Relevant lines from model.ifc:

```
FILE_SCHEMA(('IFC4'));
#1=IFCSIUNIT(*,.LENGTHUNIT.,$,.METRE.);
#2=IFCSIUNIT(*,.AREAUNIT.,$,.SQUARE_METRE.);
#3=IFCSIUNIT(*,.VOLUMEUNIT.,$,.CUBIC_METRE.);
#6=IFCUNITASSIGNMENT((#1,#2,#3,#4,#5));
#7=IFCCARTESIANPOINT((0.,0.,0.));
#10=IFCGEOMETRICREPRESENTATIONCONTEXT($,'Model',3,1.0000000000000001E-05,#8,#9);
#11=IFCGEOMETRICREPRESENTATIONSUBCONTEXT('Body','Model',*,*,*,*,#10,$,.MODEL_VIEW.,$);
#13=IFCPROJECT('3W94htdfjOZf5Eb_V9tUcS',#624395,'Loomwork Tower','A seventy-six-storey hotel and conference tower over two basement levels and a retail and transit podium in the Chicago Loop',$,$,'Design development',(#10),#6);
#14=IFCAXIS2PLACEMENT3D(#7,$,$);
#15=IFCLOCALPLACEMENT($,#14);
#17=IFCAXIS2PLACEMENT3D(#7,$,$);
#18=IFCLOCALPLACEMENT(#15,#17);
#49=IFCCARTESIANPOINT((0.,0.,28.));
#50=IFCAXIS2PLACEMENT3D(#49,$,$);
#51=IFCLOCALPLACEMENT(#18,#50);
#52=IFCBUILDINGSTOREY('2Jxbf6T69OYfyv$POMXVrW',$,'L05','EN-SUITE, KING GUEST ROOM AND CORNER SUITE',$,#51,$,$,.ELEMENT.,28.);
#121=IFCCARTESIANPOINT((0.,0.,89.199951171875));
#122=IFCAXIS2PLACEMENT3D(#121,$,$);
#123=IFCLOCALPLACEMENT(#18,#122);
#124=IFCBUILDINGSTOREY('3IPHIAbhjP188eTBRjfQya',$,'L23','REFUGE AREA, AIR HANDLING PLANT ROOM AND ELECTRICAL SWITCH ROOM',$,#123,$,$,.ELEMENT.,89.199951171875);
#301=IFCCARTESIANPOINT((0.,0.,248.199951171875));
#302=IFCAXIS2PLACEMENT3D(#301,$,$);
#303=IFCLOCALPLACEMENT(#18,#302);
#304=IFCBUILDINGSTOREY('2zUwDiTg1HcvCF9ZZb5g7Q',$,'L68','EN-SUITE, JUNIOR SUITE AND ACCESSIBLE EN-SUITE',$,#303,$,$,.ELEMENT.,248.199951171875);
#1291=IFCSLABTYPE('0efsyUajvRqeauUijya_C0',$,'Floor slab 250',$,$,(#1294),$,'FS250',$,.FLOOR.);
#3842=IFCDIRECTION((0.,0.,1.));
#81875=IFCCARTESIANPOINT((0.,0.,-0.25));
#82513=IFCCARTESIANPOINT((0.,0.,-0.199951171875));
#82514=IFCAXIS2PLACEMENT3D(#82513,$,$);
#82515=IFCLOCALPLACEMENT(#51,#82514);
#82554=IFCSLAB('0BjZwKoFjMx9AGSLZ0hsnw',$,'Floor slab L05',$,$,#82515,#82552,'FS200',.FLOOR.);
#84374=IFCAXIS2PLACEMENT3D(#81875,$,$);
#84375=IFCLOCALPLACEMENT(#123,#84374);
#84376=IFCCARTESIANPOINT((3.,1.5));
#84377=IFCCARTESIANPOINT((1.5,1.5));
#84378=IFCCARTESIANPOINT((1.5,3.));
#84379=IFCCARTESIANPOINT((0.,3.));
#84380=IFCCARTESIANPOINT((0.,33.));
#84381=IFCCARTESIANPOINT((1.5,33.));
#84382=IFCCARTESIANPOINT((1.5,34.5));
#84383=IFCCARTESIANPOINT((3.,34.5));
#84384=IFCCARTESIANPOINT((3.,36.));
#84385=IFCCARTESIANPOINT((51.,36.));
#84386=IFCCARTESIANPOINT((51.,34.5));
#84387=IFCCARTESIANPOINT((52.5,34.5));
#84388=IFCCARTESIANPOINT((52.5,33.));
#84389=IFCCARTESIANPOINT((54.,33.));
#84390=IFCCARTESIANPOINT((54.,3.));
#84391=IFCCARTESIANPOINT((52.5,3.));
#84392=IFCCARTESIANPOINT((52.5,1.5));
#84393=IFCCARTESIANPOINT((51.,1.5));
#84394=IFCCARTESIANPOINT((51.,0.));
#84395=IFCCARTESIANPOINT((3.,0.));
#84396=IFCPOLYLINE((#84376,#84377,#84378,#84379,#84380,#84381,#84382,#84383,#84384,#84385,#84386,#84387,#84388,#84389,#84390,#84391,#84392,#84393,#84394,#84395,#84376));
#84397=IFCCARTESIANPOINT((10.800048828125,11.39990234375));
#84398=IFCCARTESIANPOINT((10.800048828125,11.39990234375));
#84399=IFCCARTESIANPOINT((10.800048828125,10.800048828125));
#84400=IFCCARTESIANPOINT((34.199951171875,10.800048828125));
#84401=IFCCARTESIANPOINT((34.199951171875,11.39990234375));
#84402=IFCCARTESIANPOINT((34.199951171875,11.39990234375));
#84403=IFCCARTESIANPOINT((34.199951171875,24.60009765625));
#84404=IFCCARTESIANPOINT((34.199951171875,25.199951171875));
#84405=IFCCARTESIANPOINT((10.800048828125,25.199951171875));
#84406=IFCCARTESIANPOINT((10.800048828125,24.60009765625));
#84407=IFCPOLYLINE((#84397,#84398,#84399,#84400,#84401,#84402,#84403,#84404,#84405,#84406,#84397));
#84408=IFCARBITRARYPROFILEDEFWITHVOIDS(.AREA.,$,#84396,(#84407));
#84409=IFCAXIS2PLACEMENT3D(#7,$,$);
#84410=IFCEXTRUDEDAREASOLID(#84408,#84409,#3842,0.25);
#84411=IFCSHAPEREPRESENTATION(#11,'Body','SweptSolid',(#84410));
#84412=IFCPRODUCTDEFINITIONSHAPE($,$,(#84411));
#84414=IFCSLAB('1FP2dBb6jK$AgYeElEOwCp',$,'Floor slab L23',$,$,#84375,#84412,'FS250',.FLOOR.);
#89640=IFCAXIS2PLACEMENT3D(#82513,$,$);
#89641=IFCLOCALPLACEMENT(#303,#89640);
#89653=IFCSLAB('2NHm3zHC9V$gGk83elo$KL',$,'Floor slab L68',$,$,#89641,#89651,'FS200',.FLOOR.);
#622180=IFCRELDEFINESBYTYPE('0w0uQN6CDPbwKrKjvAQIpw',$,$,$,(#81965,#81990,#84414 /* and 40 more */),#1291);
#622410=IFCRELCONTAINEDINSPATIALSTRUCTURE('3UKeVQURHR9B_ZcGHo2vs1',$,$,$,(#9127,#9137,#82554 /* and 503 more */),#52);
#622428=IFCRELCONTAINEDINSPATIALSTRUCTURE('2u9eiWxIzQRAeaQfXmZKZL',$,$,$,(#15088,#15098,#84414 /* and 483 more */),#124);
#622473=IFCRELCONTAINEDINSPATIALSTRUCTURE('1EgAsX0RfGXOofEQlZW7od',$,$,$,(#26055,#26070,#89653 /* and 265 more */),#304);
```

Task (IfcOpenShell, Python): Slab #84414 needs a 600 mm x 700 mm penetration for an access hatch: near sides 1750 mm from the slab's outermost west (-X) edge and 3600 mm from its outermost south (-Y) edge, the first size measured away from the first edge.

```python
import numpy as np
import ifcopenshell
import ifcopenshell.api.feature
import ifcopenshell.api.geometry
import ifcopenshell.api.root
import ifcopenshell.geom
import ifcopenshell.util.placement
import ifcopenshell.util.representation
import ifcopenshell.util.shape
import ifcopenshell.util.unit

model = ifcopenshell.open("model.ifc")
unit_scale = ifcopenshell.util.unit.calculate_unit_scale(model)
settings = ifcopenshell.geom.settings()


def volume(element):
    """Net volume in cubic metres, openings subtracted."""
    shape = ifcopenshell.geom.create_shape(settings, element)
    return ifcopenshell.util.shape.get_volume(shape.geometry)


slab = model.by_id(84414)
before = volume(slab)

# Extent in the slab's own axes, in metres. The edges named are its -X and -Y sides.
slab_shape = ifcopenshell.geom.create_shape(settings, slab)
vertices = ifcopenshell.util.shape.get_vertices(slab_shape.geometry)
x_min, y_min, bottom = vertices.min(axis=0)
top = vertices[:, 2].max()

opening = ifcopenshell.api.root.create_entity(model, ifc_class="IfcOpeningElement", name="Access hatch opening", predefined_type="OPENING")
context = ifcopenshell.util.representation.get_context(model, "Model", "Body", "MODEL_VIEW")
width, depth = 0.6, 0.7
outline = [(0.0, 0.0), (width, 0.0), (width, depth), (0.0, depth), (0.0, 0.0)]
# Overshoot both faces by 50 mm so the cut is clean.
shape = ifcopenshell.api.geometry.add_slab_representation(
    model, context=context, depth=top - bottom + 0.1, polyline=outline
)
ifcopenshell.api.geometry.assign_representation(model, product=opening, representation=shape)

matrix = ifcopenshell.util.placement.get_local_placement(slab.ObjectPlacement)
matrix[:, 3] = matrix @ np.append(np.array([x_min + 1.75, y_min + 3.6, bottom - 0.05]) / unit_scale, 1.0)
ifcopenshell.api.geometry.edit_object_placement(model, product=opening, matrix=matrix, is_si=False)
ifcopenshell.api.feature.add_feature(model, feature=opening, element=slab)

after = volume(slab)

print(f"slab volume {before:.3f} -> {after:.3f} m3")

model.write("model_v2.ifc")
```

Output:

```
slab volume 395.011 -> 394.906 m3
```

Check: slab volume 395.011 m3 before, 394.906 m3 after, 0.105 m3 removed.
